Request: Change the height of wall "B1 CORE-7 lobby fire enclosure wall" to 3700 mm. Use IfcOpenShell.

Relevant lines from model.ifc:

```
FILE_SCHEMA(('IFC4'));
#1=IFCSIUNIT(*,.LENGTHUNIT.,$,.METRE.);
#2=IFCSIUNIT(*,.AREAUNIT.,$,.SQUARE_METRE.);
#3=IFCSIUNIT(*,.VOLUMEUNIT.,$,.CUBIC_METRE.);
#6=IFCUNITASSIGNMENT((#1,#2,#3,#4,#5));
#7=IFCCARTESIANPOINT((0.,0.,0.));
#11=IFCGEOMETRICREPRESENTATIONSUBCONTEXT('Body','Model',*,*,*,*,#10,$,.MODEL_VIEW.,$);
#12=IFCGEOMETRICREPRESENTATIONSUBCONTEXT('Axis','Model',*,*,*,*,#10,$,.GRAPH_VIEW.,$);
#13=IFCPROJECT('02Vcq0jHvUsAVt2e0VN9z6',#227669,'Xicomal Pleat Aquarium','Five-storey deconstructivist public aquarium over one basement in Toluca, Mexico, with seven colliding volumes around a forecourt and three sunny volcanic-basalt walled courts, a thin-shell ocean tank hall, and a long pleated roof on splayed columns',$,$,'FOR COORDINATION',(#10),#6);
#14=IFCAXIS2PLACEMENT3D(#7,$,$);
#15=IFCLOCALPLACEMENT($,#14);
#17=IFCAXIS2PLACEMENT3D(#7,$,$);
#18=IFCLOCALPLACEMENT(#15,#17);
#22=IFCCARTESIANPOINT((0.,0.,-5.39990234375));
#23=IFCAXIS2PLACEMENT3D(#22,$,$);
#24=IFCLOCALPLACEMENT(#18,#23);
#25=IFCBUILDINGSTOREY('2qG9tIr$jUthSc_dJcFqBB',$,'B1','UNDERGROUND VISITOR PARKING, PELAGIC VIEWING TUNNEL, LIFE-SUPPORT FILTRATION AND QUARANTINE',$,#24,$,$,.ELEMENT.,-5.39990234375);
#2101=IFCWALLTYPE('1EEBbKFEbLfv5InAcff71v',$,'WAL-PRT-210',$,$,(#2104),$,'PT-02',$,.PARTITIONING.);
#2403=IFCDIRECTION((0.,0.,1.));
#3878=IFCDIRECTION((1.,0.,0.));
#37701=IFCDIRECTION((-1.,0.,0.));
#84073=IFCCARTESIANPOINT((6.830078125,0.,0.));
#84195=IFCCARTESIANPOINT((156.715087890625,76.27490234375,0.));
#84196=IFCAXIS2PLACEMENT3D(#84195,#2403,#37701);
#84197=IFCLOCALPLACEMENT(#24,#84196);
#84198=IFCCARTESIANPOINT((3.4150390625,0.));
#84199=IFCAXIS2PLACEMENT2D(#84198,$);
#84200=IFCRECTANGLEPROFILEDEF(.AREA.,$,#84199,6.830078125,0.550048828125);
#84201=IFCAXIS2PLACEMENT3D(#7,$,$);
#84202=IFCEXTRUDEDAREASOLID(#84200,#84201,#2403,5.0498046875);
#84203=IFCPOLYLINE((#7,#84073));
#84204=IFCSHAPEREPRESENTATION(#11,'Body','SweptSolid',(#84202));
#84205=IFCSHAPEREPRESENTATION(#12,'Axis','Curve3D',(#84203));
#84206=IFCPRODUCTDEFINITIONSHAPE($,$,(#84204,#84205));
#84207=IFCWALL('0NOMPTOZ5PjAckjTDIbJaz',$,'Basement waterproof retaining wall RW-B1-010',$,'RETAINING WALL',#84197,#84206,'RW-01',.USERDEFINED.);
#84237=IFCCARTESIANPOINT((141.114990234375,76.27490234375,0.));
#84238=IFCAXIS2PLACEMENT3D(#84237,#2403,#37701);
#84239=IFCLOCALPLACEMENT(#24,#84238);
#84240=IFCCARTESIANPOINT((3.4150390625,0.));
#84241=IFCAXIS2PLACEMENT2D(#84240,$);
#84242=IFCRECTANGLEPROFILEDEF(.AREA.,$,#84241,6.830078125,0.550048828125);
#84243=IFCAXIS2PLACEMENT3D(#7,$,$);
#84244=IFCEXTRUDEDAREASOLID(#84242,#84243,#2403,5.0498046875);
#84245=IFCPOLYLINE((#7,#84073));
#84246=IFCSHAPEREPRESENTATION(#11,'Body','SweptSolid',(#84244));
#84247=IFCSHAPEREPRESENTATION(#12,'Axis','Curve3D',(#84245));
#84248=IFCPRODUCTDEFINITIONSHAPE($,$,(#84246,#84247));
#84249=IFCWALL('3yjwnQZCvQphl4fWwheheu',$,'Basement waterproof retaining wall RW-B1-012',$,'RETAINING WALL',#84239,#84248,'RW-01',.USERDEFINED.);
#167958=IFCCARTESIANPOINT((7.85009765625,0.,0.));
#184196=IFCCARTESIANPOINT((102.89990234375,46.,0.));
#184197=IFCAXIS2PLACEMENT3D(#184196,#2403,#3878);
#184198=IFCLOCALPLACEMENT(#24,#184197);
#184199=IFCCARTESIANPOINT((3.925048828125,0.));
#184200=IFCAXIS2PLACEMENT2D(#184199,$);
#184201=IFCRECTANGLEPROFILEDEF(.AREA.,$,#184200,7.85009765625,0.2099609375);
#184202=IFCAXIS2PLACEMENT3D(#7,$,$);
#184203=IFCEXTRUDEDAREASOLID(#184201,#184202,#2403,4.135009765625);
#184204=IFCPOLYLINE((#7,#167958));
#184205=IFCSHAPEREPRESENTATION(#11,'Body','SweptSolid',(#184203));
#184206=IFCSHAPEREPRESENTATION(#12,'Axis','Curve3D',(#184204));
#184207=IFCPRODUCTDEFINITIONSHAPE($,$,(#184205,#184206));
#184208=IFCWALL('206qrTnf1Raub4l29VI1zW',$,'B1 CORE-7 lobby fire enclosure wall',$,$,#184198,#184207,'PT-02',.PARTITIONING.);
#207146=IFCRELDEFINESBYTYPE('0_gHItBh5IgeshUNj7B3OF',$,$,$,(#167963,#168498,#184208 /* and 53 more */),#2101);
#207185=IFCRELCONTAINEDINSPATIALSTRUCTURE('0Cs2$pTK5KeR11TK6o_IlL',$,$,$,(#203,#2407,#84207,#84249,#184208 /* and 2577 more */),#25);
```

```python
import ifcopenshell
import ifcopenshell.geom
import ifcopenshell.util.representation
import ifcopenshell.util.shape
import ifcopenshell.util.unit

model = ifcopenshell.open("model.ifc")
unit_scale = ifcopenshell.util.unit.calculate_unit_scale(model)
settings = ifcopenshell.geom.settings()


def volume(element):
    """Net volume in cubic metres, openings subtracted."""
    shape = ifcopenshell.geom.create_shape(settings, element)
    return ifcopenshell.util.shape.get_volume(shape.geometry)


wall = model.by_id(184208)
before = volume(wall)

body = ifcopenshell.util.representation.get_representation(wall, "Model", "Body")
solid = body.Items[0]
old_height = solid.Depth
solid.Depth = 3.7 / unit_scale
after = volume(wall)

print(f"height {old_height:g} -> {solid.Depth:g}, volume {before:.3f} -> {after:.3f} m3")

model.write("model_v2.ifc")
```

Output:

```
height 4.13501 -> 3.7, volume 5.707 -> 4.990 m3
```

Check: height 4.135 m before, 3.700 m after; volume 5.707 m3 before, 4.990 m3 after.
